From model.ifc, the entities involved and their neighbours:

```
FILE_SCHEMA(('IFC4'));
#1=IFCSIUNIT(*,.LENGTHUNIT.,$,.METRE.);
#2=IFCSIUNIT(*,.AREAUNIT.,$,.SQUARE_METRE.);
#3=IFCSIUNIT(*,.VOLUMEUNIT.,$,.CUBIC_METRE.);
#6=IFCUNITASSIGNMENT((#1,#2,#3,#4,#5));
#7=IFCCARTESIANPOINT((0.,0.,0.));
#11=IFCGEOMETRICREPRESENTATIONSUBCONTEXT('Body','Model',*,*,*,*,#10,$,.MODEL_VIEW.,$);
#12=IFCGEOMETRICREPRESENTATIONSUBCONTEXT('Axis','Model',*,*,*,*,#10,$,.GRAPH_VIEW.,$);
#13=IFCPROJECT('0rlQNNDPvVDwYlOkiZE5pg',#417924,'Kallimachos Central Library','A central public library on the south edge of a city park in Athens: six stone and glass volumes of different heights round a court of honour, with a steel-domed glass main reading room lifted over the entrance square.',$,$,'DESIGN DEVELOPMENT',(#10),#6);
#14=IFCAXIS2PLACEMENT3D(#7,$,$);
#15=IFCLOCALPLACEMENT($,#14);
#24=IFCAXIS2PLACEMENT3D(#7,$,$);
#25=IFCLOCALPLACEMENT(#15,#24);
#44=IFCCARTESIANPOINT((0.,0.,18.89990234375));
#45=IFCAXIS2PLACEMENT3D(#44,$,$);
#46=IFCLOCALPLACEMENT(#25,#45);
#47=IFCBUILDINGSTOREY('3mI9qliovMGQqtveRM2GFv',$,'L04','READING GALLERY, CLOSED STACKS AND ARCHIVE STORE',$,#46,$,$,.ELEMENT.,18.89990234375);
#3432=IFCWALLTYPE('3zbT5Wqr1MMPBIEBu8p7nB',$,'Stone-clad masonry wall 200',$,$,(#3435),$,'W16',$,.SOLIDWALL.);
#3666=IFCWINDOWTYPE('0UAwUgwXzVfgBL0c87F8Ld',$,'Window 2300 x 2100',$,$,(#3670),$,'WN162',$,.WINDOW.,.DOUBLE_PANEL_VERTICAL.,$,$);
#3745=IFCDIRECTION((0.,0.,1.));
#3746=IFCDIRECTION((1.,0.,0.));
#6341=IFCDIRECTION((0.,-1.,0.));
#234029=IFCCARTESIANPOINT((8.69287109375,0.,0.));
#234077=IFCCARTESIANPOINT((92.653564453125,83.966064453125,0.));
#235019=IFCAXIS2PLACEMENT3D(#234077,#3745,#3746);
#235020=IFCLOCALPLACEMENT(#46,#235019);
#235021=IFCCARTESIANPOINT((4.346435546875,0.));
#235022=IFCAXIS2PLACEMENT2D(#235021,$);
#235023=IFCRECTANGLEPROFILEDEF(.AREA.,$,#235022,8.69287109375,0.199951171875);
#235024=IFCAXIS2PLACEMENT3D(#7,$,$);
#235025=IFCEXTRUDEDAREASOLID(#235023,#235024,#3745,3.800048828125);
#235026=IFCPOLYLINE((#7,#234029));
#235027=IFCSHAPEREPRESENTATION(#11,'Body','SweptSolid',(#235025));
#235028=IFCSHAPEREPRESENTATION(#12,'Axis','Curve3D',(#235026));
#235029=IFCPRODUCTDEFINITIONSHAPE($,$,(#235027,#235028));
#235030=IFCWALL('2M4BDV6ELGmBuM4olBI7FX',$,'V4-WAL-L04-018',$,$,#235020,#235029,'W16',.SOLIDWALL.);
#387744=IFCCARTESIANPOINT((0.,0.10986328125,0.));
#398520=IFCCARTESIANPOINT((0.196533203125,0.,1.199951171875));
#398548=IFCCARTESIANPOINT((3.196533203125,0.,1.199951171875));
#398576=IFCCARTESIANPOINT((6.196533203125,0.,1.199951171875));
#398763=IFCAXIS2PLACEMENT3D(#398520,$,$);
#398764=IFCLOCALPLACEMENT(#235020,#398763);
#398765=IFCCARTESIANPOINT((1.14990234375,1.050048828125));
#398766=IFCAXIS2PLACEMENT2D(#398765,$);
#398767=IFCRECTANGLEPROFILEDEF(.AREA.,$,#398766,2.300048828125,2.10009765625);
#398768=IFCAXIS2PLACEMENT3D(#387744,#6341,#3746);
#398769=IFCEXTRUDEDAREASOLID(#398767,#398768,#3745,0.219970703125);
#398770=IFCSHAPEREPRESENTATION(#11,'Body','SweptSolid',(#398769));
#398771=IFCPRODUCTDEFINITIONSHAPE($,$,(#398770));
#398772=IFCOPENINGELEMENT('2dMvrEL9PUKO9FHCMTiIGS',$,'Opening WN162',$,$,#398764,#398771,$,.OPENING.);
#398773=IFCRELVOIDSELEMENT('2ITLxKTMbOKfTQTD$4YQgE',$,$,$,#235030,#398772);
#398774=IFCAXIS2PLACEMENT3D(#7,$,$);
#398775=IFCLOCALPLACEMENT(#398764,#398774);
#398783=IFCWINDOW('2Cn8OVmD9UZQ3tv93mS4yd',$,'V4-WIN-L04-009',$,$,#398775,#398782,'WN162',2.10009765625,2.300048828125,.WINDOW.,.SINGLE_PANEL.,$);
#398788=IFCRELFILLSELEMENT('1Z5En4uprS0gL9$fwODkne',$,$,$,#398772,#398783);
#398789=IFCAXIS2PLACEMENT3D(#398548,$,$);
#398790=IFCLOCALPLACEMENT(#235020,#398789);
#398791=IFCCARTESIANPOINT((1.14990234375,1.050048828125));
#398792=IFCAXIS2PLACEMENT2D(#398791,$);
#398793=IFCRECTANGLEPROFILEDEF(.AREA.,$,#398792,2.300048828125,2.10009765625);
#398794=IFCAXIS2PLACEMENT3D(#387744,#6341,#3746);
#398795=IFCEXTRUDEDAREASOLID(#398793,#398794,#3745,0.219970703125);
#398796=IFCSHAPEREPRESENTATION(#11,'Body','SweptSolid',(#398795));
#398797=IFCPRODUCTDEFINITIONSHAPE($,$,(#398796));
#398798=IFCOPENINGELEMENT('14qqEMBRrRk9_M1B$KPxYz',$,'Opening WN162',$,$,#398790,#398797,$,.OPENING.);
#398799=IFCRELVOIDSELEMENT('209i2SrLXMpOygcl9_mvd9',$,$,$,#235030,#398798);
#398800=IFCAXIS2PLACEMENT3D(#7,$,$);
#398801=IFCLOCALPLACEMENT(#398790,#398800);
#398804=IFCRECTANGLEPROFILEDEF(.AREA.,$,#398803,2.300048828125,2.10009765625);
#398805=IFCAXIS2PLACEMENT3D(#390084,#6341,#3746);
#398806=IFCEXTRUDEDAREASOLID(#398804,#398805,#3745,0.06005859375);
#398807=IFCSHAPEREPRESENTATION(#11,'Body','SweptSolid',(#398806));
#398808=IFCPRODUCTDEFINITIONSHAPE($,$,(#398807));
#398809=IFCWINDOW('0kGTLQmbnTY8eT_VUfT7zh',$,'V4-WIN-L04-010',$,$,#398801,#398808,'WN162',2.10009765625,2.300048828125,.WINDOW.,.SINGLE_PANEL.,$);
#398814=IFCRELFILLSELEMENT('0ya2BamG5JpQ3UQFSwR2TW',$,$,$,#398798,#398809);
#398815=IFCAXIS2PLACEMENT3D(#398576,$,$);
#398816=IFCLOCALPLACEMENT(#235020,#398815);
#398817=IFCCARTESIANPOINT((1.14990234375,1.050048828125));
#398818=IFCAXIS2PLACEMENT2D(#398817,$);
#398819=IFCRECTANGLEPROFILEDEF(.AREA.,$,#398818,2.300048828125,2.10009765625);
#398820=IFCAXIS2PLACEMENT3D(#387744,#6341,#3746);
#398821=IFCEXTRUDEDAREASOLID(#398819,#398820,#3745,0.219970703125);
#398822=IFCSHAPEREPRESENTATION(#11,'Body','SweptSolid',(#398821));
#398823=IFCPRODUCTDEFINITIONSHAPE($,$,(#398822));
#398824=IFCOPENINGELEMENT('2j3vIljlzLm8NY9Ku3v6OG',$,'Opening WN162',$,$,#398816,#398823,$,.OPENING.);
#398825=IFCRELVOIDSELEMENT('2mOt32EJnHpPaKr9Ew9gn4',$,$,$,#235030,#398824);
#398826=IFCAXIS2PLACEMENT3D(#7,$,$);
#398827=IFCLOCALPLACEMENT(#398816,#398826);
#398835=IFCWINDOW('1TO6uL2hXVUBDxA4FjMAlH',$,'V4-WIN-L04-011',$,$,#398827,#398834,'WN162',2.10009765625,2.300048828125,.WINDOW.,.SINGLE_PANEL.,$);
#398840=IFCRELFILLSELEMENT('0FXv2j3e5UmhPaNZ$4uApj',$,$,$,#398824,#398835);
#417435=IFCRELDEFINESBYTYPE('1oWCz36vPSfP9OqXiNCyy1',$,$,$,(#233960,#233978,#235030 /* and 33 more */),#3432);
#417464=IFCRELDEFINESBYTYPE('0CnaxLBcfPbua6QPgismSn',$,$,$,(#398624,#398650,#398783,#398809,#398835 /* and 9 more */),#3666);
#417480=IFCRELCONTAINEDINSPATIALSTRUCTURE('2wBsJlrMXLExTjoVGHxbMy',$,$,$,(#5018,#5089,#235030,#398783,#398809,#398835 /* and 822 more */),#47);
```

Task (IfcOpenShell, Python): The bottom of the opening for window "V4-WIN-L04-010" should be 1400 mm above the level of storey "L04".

```python
import numpy as np
import ifcopenshell
import ifcopenshell.api.geometry
import ifcopenshell.geom
import ifcopenshell.util.element
import ifcopenshell.util.placement
import ifcopenshell.util.shape
import ifcopenshell.util.unit

model = ifcopenshell.open("model.ifc")
unit_scale = ifcopenshell.util.unit.calculate_unit_scale(model)

window = model.by_guid("0kGTLQmbnTY8eT_VUfT7zh")
opening = window.FillsVoids[0].RelatingOpeningElement
storey = ifcopenshell.util.element.get_container(window, ifc_class="IfcBuildingStorey")
level = ifcopenshell.util.placement.get_local_placement(storey.ObjectPlacement)[2, 3]

# The opening's origin need not be at the sill, so measure its lowest point.
shape = ifcopenshell.geom.create_shape(ifcopenshell.geom.settings(), opening)
bottom = ifcopenshell.util.shape.get_shape_bottom_elevation(shape, shape.geometry) / unit_scale
dz = level + 1.4 / unit_scale - bottom

shift = np.array([0.0, 0.0, dz])
# The window is placed relative to its opening, so it follows when the opening moves.
matrix = ifcopenshell.util.placement.get_local_placement(opening.ObjectPlacement)
matrix[:3, 3] += shift
ifcopenshell.api.geometry.edit_object_placement(
    model, product=opening, matrix=matrix, is_si=False, should_transform_children=True
)

print(f"moved by {dz * unit_scale:+.3f} m")

model.write("model_edited.ifc")
```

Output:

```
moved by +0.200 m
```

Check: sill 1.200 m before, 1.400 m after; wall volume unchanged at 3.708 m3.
